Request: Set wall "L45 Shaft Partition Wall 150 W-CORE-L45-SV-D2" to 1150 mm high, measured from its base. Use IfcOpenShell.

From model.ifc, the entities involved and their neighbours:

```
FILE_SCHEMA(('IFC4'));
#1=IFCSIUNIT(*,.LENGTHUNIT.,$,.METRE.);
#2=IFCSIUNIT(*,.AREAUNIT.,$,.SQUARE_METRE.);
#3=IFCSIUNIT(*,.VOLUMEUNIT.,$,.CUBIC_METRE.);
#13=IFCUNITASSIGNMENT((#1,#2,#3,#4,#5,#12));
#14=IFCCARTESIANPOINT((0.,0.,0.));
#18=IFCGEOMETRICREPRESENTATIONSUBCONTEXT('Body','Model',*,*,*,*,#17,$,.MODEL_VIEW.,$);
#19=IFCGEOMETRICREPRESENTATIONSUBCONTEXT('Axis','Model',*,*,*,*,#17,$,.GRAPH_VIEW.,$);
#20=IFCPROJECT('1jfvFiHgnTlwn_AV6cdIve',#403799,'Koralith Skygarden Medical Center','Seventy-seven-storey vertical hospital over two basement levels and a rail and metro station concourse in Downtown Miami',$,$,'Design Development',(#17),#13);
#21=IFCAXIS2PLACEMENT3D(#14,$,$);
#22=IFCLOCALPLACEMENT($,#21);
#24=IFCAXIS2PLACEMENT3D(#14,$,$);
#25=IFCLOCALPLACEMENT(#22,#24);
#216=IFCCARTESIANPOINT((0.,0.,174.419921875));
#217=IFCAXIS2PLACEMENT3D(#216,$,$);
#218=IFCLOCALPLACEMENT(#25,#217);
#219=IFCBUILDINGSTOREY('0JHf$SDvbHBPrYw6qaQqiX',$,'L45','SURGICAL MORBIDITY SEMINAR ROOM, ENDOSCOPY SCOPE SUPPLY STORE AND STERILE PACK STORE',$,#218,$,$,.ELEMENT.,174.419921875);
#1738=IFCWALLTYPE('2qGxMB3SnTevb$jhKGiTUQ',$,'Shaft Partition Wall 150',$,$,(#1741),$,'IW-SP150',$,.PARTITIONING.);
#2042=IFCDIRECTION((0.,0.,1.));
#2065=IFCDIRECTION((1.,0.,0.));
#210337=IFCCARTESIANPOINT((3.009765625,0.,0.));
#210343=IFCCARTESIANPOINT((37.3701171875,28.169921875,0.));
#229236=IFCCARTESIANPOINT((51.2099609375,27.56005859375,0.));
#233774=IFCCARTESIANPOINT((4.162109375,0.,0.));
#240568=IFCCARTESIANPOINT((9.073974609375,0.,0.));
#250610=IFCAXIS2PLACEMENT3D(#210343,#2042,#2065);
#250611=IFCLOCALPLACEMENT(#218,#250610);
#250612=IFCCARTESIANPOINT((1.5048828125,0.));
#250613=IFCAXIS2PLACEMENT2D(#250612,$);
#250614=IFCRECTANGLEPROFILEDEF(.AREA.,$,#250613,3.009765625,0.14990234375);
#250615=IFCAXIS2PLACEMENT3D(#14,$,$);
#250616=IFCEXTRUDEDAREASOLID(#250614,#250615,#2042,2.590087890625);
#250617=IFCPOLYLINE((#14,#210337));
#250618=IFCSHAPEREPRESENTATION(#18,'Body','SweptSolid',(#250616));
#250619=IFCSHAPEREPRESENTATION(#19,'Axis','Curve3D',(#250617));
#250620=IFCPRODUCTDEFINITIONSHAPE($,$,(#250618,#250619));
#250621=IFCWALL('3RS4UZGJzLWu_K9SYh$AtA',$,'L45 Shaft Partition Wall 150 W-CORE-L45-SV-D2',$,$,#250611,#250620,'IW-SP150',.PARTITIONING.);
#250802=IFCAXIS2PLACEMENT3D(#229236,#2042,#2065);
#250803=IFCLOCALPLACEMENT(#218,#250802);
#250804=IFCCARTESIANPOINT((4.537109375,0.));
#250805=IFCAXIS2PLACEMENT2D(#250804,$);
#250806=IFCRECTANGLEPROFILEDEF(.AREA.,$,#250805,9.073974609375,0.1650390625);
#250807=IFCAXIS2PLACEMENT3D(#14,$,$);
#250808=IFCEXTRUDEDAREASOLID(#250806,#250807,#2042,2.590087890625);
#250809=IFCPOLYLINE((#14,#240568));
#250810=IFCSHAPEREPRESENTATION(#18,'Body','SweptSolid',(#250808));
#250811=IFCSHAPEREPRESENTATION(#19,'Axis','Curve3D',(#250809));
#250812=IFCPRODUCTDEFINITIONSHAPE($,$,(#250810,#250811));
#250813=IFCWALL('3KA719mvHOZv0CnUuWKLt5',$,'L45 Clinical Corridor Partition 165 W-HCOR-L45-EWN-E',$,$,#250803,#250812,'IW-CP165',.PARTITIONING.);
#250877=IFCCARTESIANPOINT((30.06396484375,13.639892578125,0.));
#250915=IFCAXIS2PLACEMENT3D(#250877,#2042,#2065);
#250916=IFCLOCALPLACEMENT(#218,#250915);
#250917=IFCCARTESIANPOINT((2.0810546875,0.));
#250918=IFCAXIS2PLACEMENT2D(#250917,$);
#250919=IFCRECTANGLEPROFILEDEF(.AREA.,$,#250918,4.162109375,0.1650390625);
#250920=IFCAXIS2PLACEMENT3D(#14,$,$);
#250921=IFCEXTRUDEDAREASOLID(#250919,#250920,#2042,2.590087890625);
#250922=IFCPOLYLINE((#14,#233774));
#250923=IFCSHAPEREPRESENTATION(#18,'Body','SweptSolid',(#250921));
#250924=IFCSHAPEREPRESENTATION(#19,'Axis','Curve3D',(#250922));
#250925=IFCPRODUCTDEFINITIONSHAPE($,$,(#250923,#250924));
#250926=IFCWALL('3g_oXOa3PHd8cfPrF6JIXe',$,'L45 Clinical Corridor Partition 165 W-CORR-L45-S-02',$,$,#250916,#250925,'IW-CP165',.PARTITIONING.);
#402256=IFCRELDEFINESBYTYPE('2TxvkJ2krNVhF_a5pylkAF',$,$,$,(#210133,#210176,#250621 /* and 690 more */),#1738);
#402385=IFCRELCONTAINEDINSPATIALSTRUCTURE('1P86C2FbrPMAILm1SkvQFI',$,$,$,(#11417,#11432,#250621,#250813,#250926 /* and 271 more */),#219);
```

```python
import ifcopenshell
import ifcopenshell.geom
import ifcopenshell.util.representation
import ifcopenshell.util.shape
import ifcopenshell.util.unit

model = ifcopenshell.open("model.ifc")
unit_scale = ifcopenshell.util.unit.calculate_unit_scale(model)
settings = ifcopenshell.geom.settings()


def volume(element):
    """Net volume in cubic metres, openings subtracted."""
    shape = ifcopenshell.geom.create_shape(settings, element)
    return ifcopenshell.util.shape.get_volume(shape.geometry)


wall = model.by_guid("3RS4UZGJzLWu_K9SYh$AtA")
before = volume(wall)

body = ifcopenshell.util.representation.get_representation(wall, "Model", "Body")
solid = body.Items[0]
old_height = solid.Depth
solid.Depth = 1.15 / unit_scale
after = volume(wall)

print(f"height {old_height:g} -> {solid.Depth:g}, volume {before:.3f} -> {after:.3f} m3")

model.write("model_v2.ifc")
```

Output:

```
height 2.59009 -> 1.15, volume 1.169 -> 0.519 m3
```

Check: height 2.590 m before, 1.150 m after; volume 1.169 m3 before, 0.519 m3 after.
